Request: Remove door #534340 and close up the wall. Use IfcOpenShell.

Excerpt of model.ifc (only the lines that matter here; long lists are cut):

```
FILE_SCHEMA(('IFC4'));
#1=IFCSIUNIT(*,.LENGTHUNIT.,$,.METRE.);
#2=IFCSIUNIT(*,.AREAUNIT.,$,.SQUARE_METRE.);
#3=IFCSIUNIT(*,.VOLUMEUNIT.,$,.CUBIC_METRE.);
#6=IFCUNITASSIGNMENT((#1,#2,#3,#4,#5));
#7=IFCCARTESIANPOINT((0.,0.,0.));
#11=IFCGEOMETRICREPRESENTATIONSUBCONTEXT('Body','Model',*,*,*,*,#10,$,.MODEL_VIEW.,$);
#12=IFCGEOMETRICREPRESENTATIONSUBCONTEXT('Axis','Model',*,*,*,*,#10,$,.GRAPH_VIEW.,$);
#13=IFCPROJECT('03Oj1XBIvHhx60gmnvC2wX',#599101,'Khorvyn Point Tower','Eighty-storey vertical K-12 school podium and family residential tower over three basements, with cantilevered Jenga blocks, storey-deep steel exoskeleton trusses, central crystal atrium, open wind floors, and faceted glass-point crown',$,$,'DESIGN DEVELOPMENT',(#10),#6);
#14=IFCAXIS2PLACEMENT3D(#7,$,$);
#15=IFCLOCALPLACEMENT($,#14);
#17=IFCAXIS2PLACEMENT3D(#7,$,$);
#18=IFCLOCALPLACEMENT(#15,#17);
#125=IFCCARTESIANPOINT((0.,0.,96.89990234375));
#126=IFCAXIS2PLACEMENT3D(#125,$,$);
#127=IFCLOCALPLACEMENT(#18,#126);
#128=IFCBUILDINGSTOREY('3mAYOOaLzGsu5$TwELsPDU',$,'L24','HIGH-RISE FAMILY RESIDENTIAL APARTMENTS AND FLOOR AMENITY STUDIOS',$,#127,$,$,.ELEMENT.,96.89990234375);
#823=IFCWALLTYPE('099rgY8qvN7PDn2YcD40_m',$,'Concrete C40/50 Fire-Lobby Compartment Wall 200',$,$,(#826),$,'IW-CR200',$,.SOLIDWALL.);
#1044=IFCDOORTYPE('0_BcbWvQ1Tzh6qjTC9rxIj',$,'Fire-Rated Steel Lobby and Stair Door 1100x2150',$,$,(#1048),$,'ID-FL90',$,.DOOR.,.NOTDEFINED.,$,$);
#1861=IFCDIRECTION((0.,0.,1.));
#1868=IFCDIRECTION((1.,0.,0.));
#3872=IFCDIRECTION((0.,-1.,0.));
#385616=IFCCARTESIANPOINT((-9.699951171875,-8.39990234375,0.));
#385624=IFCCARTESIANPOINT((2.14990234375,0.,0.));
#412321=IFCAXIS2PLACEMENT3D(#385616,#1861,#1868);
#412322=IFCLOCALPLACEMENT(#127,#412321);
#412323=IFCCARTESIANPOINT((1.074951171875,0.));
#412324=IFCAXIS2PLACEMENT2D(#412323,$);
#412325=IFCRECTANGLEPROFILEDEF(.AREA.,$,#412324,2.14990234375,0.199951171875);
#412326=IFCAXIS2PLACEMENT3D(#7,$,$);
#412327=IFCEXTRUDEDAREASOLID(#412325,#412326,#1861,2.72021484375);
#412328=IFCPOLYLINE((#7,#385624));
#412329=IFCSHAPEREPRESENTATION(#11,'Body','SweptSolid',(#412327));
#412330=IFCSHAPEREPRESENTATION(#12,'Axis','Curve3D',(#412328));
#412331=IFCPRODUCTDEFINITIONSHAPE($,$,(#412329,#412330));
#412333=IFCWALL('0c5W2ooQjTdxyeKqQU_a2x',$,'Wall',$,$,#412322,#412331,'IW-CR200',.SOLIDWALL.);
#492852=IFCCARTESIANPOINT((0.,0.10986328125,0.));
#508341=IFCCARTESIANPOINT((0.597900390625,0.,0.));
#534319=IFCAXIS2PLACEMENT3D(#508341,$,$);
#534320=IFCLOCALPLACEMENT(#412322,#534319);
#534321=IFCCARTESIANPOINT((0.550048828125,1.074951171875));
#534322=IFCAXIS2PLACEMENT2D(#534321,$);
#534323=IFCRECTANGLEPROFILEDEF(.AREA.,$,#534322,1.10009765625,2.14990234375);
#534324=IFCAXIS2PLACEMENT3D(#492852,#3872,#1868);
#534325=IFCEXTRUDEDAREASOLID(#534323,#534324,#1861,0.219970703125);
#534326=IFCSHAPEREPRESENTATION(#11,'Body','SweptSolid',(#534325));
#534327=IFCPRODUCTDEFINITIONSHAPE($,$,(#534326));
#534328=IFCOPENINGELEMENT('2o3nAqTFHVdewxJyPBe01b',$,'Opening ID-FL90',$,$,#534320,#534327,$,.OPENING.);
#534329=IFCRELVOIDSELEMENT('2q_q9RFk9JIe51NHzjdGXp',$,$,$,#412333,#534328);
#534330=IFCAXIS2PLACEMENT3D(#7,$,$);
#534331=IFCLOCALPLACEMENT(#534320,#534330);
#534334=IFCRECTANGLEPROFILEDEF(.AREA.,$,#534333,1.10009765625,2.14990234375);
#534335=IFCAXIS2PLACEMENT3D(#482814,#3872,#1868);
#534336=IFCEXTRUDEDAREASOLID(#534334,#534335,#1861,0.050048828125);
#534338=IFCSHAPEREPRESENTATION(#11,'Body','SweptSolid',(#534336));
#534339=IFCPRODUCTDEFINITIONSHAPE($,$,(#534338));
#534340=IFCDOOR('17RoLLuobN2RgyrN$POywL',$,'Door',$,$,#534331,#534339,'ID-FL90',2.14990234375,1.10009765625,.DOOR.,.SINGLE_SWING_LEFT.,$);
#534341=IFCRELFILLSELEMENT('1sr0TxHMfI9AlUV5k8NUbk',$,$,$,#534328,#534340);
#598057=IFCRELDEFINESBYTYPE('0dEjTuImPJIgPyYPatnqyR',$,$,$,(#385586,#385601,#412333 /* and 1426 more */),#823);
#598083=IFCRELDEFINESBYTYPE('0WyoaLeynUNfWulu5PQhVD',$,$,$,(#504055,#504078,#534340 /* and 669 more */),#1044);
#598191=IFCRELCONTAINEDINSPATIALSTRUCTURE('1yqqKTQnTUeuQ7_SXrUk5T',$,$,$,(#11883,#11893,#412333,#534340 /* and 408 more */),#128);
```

```python
import ifcopenshell
import ifcopenshell.api.feature
import ifcopenshell.api.root
import ifcopenshell.geom
import ifcopenshell.util.shape

model = ifcopenshell.open("model.ifc")
settings = ifcopenshell.geom.settings()


def volume(element):
    """Net volume in cubic metres, openings subtracted."""
    shape = ifcopenshell.geom.create_shape(settings, element)
    return ifcopenshell.util.shape.get_volume(shape.geometry)


door = model.by_guid("17RoLLuobN2RgyrN$POywL")
opening = door.FillsVoids[0].RelatingOpeningElement
wall = opening.VoidsElements[0].RelatingBuildingElement
before = volume(wall)

ifcopenshell.api.root.remove_product(model, product=door)
ifcopenshell.api.feature.remove_feature(model, feature=opening)

after = volume(wall)

print(f"wall volume {before:.3f} -> {after:.3f} m3")

model.write("model_edited.ifc")
```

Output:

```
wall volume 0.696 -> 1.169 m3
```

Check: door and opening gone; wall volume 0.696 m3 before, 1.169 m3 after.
